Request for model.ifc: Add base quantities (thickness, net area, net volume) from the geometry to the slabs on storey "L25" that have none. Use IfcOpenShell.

First a look at what the model holds.

```python
import ifcopenshell
import ifcopenshell.util.element
import ifcopenshell.util.unit

model = ifcopenshell.open("model.ifc")
print(model.schema)
for unit_type in ("LENGTHUNIT", "AREAUNIT", "VOLUMEUNIT"):
    print(unit_type, ifcopenshell.util.unit.calculate_unit_scale(model, unit_type))
storey = next(s for s in model.by_type("IfcBuildingStorey") if s.Name == "L25")
slabs = [e for e in ifcopenshell.util.element.get_decomposition(storey) if e.is_a("IfcSlab")]
for e in sorted(slabs, key=lambda e: e.id()):
    print(e.id(), e.is_a(), e.Name, list(ifcopenshell.util.element.get_psets(e, qtos_only=True)), sep=" | ")
```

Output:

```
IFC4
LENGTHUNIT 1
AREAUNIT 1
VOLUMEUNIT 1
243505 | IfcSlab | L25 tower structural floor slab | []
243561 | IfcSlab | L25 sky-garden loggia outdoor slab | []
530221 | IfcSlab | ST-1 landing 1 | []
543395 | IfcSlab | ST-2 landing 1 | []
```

```python
import ifcopenshell
import ifcopenshell.api.pset
import ifcopenshell.geom
import ifcopenshell.util.element
import ifcopenshell.util.shape
import ifcopenshell.util.unit

model = ifcopenshell.open("model.ifc")
unit_scale = ifcopenshell.util.unit.calculate_unit_scale(model)
area_scale = ifcopenshell.util.unit.calculate_unit_scale(model, "AREAUNIT")
volume_scale = ifcopenshell.util.unit.calculate_unit_scale(model, "VOLUMEUNIT")
settings = ifcopenshell.geom.settings()

storey = next(s for s in model.by_type("IfcBuildingStorey") if s.Name == "L25")
slabs = [e for e in ifcopenshell.util.element.get_decomposition(storey) if e.is_a("IfcSlab")]

for e in sorted(slabs, key=lambda e: e.id()):
    if ifcopenshell.util.element.get_psets(e, qtos_only=True, should_inherit=False):
        continue
    # Geometry comes back in metres, in the element's own axes.
    shape = ifcopenshell.geom.create_shape(settings, e)
    values = {
        "Width": ifcopenshell.util.shape.get_z(shape.geometry) / unit_scale,
        "NetArea": ifcopenshell.util.shape.get_footprint_area(shape.geometry) / area_scale,
        "NetVolume": ifcopenshell.util.shape.get_volume(shape.geometry) / volume_scale,
    }
    qto = ifcopenshell.api.pset.add_qto(model, product=e, name="Qto_SlabBaseQuantities")
    ifcopenshell.api.pset.edit_qto(model, qto=qto, properties=values)
    print(e.id(), {k: round(v, 3) for k, v in values.items()})

model.write("model_rev.ifc")
```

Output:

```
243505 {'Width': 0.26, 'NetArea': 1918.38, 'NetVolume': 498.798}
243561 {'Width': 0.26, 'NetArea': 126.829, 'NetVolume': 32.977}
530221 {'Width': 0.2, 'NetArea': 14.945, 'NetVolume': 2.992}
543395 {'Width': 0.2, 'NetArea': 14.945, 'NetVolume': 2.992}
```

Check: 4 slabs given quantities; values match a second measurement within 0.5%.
